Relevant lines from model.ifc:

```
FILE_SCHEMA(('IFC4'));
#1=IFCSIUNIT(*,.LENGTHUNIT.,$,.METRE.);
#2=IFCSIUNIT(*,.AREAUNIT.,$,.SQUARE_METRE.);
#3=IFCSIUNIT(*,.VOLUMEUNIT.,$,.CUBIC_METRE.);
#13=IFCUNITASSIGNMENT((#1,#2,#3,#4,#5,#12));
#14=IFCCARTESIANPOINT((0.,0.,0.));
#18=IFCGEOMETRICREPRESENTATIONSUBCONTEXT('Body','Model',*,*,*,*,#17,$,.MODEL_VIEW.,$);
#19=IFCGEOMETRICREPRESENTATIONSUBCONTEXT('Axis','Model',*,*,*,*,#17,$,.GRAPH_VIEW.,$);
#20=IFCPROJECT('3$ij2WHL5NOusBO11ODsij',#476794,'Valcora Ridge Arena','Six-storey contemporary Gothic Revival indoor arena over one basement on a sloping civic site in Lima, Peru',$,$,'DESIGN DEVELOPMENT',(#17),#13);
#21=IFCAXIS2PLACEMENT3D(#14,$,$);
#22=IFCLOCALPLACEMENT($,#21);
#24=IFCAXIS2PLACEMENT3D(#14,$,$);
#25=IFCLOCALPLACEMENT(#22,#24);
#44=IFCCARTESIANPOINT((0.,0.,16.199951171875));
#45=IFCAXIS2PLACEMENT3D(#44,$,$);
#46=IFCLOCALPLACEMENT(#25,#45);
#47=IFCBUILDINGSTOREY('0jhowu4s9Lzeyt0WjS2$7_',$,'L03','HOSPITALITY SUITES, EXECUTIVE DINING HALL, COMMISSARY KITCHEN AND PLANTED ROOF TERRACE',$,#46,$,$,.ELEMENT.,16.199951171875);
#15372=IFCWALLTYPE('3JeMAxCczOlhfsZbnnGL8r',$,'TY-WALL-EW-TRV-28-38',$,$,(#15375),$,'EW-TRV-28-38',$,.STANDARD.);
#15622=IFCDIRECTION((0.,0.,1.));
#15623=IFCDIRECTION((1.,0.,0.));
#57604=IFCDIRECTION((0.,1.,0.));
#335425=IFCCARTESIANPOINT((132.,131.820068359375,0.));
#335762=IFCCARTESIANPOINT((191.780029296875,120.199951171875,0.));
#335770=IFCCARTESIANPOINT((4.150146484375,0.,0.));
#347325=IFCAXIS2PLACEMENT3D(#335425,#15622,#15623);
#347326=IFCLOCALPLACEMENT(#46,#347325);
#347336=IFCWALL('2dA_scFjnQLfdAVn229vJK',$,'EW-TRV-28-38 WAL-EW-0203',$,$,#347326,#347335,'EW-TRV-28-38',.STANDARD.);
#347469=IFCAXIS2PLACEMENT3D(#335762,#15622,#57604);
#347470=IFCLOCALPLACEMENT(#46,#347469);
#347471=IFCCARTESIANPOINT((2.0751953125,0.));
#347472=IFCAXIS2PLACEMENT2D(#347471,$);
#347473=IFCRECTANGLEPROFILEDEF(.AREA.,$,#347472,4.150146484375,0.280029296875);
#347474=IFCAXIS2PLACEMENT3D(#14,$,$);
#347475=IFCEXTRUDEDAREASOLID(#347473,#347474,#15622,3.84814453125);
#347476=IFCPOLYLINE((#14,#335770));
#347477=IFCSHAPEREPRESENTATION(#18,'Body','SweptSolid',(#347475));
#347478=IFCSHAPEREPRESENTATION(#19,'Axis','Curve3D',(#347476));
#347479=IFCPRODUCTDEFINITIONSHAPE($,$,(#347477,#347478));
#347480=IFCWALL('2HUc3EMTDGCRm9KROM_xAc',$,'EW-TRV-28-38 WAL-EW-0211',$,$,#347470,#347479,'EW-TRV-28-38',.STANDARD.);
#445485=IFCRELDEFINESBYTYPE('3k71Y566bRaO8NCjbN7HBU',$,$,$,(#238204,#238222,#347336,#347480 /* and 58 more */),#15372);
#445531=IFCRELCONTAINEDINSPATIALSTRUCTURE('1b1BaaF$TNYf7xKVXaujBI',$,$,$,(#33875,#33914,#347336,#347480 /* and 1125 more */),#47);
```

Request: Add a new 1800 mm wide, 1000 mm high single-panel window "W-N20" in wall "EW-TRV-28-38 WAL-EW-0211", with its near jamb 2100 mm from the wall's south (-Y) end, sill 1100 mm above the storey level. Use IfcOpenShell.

```python
import numpy as np
import ifcopenshell
import ifcopenshell.api.feature
import ifcopenshell.api.geometry
import ifcopenshell.api.root
import ifcopenshell.api.spatial
import ifcopenshell.geom
import ifcopenshell.util.element
import ifcopenshell.util.placement
import ifcopenshell.util.representation
import ifcopenshell.util.shape
import ifcopenshell.util.unit

model = ifcopenshell.open("model.ifc")
unit_scale = ifcopenshell.util.unit.calculate_unit_scale(model)
settings = ifcopenshell.geom.settings()


def volume(element):
    """Net volume in cubic metres, openings subtracted."""
    shape = ifcopenshell.geom.create_shape(settings, element)
    return ifcopenshell.util.shape.get_volume(shape.geometry)


wall = model.by_id(347480)
storey = ifcopenshell.util.element.get_container(wall, ifc_class="IfcBuildingStorey")
context = ifcopenshell.util.representation.get_context(model, "Model", "Body", "MODEL_VIEW")
before = volume(wall)

width, height, from_end, sill = 1.8, 1, 2.1, 1.1  # metres

# The wall runs along its own X axis, and the end named is its -X end.
wall_shape = ifcopenshell.geom.create_shape(settings, wall)
x, y, z = ifcopenshell.util.shape.get_vertices(wall_shape.geometry).T
start = x.min() + from_end
face, thickness = float(y.min()), float(y.max() - y.min())
wall_matrix = ifcopenshell.util.placement.get_local_placement(wall.ObjectPlacement)
level = ifcopenshell.util.placement.get_local_placement(storey.ObjectPlacement)[2, 3]


def in_wall(x, y):
    """Placement at x, y metres in the wall's axes, at sill height."""
    matrix = wall_matrix.copy()
    matrix[:, 3] = wall_matrix @ np.array([x / unit_scale, y / unit_scale, 0.0, 1.0])
    matrix[2, 3] = level + sill / unit_scale
    return matrix


# Opening: a box that overshoots both wall faces by 50 mm.
opening = ifcopenshell.api.root.create_entity(model, ifc_class="IfcOpeningElement", predefined_type="OPENING")
box = ifcopenshell.api.geometry.add_wall_representation(
    model, context=context, length=width, height=height, thickness=thickness + 0.1
)
ifcopenshell.api.geometry.assign_representation(model, product=opening, representation=box)
ifcopenshell.api.geometry.edit_object_placement(model, product=opening, matrix=in_wall(start, face - 0.05), is_si=False)
ifcopenshell.api.feature.add_feature(model, feature=opening, element=wall)

window = ifcopenshell.api.root.create_entity(model, ifc_class="IfcWindow", name="W-N20", predefined_type="WINDOW")
window.OverallWidth, window.OverallHeight = width / unit_scale, height / unit_scale
window.PartitioningType = "SINGLE_PANEL"
body = ifcopenshell.api.geometry.add_window_representation(
    model,
    context=context,
    overall_width=window.OverallWidth,
    overall_height=window.OverallHeight,
    partition_type="SINGLE_PANEL",
)
ifcopenshell.api.geometry.assign_representation(model, product=window, representation=body)
ifcopenshell.api.spatial.assign_container(model, products=[window], relating_structure=storey)
ifcopenshell.api.feature.add_filling(model, opening=opening, element=window)

# Centre the window in the wall's thickness.
ifcopenshell.api.geometry.edit_object_placement(model, product=window, matrix=in_wall(start, face), is_si=False)
window_shape = ifcopenshell.geom.create_shape(settings, window)
depth = ifcopenshell.util.shape.get_vertices(window_shape.geometry)[:, 1]
offset = face + thickness / 2 - (depth.min() + depth.max()) / 2
ifcopenshell.api.geometry.edit_object_placement(model, product=window, matrix=in_wall(start, offset), is_si=False)

after = volume(wall)

print(f"wall volume {before:.3f} -> {after:.3f} m3")

model.write("model_v2.ifc")
```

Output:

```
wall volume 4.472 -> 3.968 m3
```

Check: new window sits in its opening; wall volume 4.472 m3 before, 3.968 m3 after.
